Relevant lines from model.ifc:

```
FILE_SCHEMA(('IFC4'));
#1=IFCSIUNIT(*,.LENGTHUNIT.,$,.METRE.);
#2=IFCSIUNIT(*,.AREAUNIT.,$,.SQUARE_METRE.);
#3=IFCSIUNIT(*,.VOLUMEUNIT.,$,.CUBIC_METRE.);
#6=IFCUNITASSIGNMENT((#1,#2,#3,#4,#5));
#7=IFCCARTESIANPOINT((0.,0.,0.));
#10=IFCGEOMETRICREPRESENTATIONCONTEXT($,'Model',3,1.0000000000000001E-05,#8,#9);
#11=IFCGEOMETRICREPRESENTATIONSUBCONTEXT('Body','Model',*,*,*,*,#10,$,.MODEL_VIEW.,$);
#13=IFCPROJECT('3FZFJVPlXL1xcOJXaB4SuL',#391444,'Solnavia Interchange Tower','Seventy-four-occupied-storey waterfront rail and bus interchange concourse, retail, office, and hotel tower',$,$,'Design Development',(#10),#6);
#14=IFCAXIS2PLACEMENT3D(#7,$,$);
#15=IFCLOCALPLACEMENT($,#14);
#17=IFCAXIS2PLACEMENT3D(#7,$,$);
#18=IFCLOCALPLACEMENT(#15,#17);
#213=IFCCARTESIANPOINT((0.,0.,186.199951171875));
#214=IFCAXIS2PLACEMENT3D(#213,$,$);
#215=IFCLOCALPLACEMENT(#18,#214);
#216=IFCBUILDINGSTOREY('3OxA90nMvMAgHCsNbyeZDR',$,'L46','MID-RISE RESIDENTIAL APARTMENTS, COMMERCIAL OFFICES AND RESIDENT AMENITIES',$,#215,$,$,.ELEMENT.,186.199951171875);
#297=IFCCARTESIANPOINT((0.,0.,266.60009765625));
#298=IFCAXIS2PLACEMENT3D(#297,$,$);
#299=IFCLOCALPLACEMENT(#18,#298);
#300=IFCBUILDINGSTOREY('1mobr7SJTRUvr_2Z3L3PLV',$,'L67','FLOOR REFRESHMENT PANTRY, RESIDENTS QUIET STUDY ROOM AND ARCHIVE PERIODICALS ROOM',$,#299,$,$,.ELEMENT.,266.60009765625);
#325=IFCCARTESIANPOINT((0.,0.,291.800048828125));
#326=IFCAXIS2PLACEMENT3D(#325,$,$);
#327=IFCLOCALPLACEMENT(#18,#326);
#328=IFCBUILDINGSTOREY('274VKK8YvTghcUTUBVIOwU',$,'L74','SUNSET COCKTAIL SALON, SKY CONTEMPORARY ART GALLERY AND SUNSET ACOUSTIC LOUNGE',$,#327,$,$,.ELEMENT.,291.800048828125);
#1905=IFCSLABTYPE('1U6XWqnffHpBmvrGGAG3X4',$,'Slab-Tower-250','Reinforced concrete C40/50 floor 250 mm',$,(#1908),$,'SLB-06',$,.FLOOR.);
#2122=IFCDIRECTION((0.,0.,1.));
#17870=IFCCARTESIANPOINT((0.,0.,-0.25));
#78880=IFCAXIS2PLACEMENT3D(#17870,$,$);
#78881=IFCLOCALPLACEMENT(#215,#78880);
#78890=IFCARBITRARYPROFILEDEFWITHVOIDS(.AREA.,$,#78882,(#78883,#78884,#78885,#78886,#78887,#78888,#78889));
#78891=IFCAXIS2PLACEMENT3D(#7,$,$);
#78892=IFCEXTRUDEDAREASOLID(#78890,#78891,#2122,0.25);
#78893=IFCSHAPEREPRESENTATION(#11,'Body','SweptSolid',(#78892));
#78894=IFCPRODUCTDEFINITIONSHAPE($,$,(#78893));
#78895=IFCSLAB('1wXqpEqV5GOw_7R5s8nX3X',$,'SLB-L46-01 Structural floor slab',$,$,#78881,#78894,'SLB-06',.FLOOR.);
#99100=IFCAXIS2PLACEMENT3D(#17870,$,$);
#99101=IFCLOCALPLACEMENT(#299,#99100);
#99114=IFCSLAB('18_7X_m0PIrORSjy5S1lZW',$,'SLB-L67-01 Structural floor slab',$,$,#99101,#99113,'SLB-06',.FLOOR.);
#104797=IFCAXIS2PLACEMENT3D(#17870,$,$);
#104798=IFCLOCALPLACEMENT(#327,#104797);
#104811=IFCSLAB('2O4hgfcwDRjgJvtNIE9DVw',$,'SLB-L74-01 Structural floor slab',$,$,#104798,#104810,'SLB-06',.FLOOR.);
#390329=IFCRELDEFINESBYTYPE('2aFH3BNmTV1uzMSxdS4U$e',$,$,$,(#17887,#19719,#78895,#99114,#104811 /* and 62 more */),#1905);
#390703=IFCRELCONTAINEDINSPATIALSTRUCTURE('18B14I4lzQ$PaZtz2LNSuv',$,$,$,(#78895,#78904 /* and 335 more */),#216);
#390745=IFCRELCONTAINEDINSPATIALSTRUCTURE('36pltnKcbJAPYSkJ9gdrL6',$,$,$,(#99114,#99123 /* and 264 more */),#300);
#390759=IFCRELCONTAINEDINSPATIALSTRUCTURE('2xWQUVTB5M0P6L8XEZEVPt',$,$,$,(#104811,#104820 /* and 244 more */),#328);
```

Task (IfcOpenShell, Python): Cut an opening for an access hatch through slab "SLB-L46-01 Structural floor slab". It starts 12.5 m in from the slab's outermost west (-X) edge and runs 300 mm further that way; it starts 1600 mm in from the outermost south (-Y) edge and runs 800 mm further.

```python
import numpy as np
import ifcopenshell
import ifcopenshell.api.feature
import ifcopenshell.api.geometry
import ifcopenshell.api.root
import ifcopenshell.geom
import ifcopenshell.util.placement
import ifcopenshell.util.representation
import ifcopenshell.util.shape
import ifcopenshell.util.unit

model = ifcopenshell.open("model.ifc")
unit_scale = ifcopenshell.util.unit.calculate_unit_scale(model)
settings = ifcopenshell.geom.settings()


def volume(element):
    """Net volume in cubic metres, openings subtracted."""
    shape = ifcopenshell.geom.create_shape(settings, element)
    return ifcopenshell.util.shape.get_volume(shape.geometry)


slab = model.by_guid("1wXqpEqV5GOw_7R5s8nX3X")
before = volume(slab)

# Extent in the slab's own axes, in metres. The edges named are its -X and -Y sides.
slab_shape = ifcopenshell.geom.create_shape(settings, slab)
vertices = ifcopenshell.util.shape.get_vertices(slab_shape.geometry)
x_min, y_min, bottom = vertices.min(axis=0)
top = vertices[:, 2].max()

opening = ifcopenshell.api.root.create_entity(model, ifc_class="IfcOpeningElement", name="Access hatch opening", predefined_type="OPENING")
context = ifcopenshell.util.representation.get_context(model, "Model", "Body", "MODEL_VIEW")
width, depth = 0.3, 0.8
outline = [(0.0, 0.0), (width, 0.0), (width, depth), (0.0, depth), (0.0, 0.0)]
# Overshoot both faces by 50 mm so the cut is clean.
shape = ifcopenshell.api.geometry.add_slab_representation(
    model, context=context, depth=top - bottom + 0.1, polyline=outline
)
ifcopenshell.api.geometry.assign_representation(model, product=opening, representation=shape)

matrix = ifcopenshell.util.placement.get_local_placement(slab.ObjectPlacement)
matrix[:, 3] = matrix @ np.append(np.array([x_min + 12.5, y_min + 1.6, bottom - 0.05]) / unit_scale, 1.0)
ifcopenshell.api.geometry.edit_object_placement(model, product=opening, matrix=matrix, is_si=False)
ifcopenshell.api.feature.add_feature(model, feature=opening, element=slab)

after = volume(slab)

print(f"slab volume {before:.3f} -> {after:.3f} m3")

model.write("model_edited.ifc")
```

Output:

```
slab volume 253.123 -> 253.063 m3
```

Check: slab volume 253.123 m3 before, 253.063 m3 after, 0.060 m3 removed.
